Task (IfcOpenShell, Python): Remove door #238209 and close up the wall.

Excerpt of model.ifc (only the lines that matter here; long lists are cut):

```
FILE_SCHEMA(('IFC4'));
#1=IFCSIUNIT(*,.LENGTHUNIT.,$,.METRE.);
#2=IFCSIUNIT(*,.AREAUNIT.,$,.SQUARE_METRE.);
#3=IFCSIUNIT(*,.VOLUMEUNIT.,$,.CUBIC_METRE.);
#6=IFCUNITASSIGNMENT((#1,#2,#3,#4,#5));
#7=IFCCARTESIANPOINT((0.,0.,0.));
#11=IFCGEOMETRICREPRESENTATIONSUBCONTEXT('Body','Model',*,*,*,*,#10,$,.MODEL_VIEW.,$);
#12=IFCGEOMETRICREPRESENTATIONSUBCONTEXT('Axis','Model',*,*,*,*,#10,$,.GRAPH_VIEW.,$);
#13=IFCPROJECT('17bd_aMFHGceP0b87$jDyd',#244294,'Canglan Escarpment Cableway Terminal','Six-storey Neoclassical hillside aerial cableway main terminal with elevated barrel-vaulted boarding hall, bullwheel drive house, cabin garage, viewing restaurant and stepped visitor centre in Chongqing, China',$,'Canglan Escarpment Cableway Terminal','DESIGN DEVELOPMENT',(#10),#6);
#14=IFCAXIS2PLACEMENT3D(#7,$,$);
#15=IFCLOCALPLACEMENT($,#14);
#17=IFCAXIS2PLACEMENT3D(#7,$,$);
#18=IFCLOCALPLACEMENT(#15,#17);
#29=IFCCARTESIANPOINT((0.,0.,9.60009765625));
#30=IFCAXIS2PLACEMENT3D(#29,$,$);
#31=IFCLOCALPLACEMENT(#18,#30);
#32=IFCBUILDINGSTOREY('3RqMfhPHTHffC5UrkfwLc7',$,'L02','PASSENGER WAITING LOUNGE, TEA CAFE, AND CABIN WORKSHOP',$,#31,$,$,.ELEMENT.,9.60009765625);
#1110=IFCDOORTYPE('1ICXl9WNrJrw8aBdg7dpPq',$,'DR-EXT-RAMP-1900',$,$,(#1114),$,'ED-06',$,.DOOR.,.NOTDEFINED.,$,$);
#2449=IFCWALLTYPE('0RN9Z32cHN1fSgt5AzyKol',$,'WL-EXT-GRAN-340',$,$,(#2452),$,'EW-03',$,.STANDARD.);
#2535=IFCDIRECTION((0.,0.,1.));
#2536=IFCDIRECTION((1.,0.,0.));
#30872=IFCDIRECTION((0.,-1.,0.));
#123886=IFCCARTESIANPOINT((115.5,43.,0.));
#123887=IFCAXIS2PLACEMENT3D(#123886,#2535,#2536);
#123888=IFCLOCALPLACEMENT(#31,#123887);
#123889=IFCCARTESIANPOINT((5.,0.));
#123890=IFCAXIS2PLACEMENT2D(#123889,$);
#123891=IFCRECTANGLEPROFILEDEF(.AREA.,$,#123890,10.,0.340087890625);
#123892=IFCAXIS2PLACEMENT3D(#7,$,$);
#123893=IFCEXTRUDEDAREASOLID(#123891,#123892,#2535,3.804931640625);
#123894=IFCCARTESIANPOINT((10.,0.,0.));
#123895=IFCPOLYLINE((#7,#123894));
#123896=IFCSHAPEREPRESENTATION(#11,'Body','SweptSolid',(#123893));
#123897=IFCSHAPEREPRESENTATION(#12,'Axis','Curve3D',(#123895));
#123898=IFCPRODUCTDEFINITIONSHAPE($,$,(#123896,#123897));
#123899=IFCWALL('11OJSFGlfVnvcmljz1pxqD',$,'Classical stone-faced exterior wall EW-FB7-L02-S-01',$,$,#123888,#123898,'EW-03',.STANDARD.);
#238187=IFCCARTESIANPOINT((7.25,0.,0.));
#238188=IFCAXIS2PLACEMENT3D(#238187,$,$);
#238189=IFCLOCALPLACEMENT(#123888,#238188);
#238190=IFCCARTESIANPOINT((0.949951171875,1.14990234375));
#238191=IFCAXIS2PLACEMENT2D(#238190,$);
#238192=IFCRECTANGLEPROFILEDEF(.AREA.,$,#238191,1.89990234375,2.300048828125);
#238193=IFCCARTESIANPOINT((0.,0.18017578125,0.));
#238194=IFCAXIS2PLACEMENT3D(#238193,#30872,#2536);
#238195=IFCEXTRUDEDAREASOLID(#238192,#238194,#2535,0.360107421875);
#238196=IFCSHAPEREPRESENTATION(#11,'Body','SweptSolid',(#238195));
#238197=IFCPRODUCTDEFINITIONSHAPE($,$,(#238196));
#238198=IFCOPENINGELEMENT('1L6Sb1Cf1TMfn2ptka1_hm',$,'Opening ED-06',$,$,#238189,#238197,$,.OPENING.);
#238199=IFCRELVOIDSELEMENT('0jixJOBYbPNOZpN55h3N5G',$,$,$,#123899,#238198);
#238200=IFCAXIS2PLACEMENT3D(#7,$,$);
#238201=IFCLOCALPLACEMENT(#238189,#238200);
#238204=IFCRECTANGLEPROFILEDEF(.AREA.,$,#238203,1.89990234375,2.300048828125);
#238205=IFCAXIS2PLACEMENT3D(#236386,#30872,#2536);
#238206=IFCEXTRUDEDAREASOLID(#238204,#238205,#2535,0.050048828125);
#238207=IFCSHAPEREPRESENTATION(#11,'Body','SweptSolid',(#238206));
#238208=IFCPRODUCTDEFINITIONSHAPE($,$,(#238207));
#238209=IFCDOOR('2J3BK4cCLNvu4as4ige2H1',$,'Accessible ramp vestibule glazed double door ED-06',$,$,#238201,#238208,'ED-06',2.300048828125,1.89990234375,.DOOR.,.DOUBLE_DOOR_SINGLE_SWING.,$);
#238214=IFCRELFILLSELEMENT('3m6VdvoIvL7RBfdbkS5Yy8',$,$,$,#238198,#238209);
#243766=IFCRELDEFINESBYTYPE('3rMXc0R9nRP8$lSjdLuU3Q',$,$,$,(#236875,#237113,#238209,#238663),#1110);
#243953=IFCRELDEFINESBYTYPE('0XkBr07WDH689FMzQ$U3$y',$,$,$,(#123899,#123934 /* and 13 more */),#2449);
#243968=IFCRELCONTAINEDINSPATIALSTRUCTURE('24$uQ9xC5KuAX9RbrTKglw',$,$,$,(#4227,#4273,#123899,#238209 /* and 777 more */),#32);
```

```python
import ifcopenshell
import ifcopenshell.api.feature
import ifcopenshell.api.root
import ifcopenshell.geom
import ifcopenshell.util.shape

model = ifcopenshell.open("model.ifc")
settings = ifcopenshell.geom.settings()


def volume(element):
    """Net volume in cubic metres, openings subtracted."""
    shape = ifcopenshell.geom.create_shape(settings, element)
    return ifcopenshell.util.shape.get_volume(shape.geometry)


door = model.by_guid("2J3BK4cCLNvu4as4ige2H1")
opening = door.FillsVoids[0].RelatingOpeningElement
wall = opening.VoidsElements[0].RelatingBuildingElement
before = volume(wall)

ifcopenshell.api.root.remove_product(model, product=door)
ifcopenshell.api.feature.remove_feature(model, feature=opening)

after = volume(wall)

print(f"wall volume {before:.3f} -> {after:.3f} m3")

model.write("model_v2.ifc")
```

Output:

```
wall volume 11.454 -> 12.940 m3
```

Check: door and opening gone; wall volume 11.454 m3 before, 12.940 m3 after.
